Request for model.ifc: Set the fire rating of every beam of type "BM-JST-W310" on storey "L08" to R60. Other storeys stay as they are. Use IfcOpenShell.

First a look at what the model holds.

```python
import ifcopenshell
import ifcopenshell.util.element

model = ifcopenshell.open("model.ifc")
print(model.schema)
storey = next(s for s in model.by_type("IfcBuildingStorey") if s.Name == "L08")
beams = [e for e in ifcopenshell.util.element.get_decomposition(storey) if e.is_a("IfcBeam")]
seen = {}
for e in beams:
    element_type = ifcopenshell.util.element.get_type(e)
    key = (element_type.Name if element_type != e and element_type else None, ifcopenshell.util.element.get_pset(e, "Pset_BeamCommon", "FireRating"))
    seen[key] = seen.get(key, 0) + 1
for (name, value), count in sorted(seen.items(), key=str):
    print(count, "x", name, "|", value)
```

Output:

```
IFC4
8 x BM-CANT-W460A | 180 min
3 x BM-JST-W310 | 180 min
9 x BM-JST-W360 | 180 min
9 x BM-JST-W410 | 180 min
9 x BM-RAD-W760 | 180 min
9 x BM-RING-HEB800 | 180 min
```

```python
import ifcopenshell
import ifcopenshell.api.pset
import ifcopenshell.util.element

model = ifcopenshell.open("model.ifc")

storey = next(s for s in model.by_type("IfcBuildingStorey") if s.Name == "L08")
beams = [e for e in ifcopenshell.util.element.get_decomposition(storey) if e.is_a("IfcBeam")]

count = 0
for e in beams:
    element_type = ifcopenshell.util.element.get_type(e)
    if element_type in (None, e) or element_type.Name != "BM-JST-W310":
        continue
    # add_pset returns the element's existing set when there is one.
    pset = ifcopenshell.api.pset.add_pset(model, product=e, name="Pset_BeamCommon")
    ifcopenshell.api.pset.edit_pset(model, pset=pset, properties={"FireRating": "R60"})
    count += 1

print(count, "beams updated")

model.write("model_v2.ifc")
```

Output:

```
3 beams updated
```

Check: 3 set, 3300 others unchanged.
